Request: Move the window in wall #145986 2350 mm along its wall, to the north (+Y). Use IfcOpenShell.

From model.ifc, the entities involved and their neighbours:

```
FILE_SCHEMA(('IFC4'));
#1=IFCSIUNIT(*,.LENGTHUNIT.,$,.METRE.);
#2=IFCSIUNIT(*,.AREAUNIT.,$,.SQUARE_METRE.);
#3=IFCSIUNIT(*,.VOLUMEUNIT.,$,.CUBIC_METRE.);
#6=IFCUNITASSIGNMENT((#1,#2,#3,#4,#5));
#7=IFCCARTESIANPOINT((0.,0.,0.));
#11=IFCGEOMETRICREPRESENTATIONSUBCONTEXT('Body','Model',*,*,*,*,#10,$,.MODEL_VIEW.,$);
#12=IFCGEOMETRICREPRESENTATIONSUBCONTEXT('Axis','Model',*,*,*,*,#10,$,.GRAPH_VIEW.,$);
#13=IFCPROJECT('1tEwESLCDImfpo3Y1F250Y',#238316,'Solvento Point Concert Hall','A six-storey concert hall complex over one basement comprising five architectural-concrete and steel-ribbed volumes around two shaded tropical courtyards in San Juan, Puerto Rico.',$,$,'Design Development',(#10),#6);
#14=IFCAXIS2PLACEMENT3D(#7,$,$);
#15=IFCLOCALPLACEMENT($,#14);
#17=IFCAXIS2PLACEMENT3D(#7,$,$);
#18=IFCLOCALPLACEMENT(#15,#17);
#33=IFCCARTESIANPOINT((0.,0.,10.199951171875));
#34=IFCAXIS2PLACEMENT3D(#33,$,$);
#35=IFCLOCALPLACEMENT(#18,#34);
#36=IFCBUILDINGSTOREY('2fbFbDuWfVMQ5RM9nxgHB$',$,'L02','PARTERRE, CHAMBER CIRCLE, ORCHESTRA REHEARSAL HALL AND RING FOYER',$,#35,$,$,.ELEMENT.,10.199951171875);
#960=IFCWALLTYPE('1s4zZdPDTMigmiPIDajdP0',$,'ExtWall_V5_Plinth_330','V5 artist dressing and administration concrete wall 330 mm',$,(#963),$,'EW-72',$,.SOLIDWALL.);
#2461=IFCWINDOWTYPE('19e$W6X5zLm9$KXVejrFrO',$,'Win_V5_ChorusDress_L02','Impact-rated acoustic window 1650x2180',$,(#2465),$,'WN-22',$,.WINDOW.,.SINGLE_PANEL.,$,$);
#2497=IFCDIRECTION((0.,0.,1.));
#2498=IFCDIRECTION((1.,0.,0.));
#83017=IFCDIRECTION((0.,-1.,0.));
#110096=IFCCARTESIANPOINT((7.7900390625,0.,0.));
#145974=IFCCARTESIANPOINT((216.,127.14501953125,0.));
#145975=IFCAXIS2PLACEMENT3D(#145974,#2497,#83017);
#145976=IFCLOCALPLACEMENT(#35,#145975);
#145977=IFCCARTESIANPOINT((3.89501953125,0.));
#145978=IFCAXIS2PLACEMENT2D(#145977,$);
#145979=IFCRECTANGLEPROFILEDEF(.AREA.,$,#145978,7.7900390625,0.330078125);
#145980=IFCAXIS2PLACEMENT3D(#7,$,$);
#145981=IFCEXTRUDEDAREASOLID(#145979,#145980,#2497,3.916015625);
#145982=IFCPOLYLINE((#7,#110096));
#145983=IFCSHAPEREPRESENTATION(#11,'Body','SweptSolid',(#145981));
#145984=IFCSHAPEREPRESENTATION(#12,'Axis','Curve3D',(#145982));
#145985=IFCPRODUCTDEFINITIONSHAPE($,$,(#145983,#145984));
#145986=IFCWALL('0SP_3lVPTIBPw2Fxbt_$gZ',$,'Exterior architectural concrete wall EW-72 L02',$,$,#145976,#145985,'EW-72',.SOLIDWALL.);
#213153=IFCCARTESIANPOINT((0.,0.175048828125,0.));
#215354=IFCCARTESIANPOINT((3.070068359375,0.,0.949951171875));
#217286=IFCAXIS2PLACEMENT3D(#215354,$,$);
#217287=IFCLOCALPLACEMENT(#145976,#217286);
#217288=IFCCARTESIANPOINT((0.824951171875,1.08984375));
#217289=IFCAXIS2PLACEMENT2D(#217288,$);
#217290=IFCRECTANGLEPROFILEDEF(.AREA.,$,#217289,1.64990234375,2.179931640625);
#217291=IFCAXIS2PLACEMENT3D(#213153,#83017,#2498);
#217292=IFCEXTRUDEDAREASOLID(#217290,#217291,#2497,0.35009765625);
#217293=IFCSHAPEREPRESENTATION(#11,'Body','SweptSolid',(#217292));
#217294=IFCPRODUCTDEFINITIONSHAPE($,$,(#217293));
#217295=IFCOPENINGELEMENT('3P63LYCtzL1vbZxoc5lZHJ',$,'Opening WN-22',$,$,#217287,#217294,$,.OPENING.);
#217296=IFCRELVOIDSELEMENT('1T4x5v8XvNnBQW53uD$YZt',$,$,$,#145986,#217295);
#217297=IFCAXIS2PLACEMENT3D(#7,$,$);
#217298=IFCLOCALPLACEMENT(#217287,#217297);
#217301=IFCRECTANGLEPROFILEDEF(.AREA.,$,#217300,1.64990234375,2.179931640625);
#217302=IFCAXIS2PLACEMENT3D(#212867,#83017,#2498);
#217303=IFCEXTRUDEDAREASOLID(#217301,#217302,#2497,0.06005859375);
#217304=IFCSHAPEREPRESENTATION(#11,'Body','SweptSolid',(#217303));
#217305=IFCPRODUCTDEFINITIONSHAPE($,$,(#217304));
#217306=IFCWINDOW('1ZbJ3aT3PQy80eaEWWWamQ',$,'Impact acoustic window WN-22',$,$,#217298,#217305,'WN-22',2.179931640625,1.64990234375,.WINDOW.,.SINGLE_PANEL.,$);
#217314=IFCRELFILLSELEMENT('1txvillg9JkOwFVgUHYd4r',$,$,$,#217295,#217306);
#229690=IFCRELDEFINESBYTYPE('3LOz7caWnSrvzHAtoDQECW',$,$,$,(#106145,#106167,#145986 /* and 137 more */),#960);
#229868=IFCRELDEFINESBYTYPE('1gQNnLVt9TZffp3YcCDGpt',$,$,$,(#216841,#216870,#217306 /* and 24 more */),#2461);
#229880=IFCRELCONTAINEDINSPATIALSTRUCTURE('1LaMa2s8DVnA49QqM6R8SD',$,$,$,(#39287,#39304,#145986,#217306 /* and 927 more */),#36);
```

```python
import ifcopenshell
import ifcopenshell.api.geometry
import ifcopenshell.util.placement

model = ifcopenshell.open("model.ifc")

window = model.by_guid("1ZbJ3aT3PQy80eaEWWWamQ")
opening = window.FillsVoids[0].RelatingOpeningElement
wall = opening.VoidsElements[0].RelatingBuildingElement

wall_matrix = ifcopenshell.util.placement.get_local_placement(wall.ObjectPlacement)
shift = wall_matrix[:3, 0] * -2.35
before = ifcopenshell.util.placement.get_local_placement(window.ObjectPlacement)[:3, 3].copy()

# The window is placed relative to its opening, so it follows when the opening moves.
matrix = ifcopenshell.util.placement.get_local_placement(opening.ObjectPlacement)
matrix[:3, 3] += shift
ifcopenshell.api.geometry.edit_object_placement(
    model, product=opening, matrix=matrix, is_si=False, should_transform_children=True
)

after = ifcopenshell.util.placement.get_local_placement(window.ObjectPlacement)[:3, 3]
print("window moved by", (after - before).round(3) + 0.0)

model.write("model_v2.ifc")
```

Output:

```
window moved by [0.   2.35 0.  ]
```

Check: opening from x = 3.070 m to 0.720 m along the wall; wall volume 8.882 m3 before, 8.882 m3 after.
